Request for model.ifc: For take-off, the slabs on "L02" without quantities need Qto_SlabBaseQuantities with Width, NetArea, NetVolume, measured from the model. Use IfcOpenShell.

First a look at what the model holds.

```python
import ifcopenshell
import ifcopenshell.util.element
import ifcopenshell.util.unit

model = ifcopenshell.open("model.ifc")
print(model.schema)
for unit_type in ("LENGTHUNIT", "AREAUNIT", "VOLUMEUNIT"):
    print(unit_type, ifcopenshell.util.unit.calculate_unit_scale(model, unit_type))
storey = next(s for s in model.by_type("IfcBuildingStorey") if s.Name == "L02")
slabs = [e for e in ifcopenshell.util.element.get_decomposition(storey) if e.is_a("IfcSlab")]
for e in sorted(slabs, key=lambda e: e.id()):
    print(e.id(), e.is_a(), e.Name, list(ifcopenshell.util.element.get_psets(e, qtos_only=True)), sep=" | ")
```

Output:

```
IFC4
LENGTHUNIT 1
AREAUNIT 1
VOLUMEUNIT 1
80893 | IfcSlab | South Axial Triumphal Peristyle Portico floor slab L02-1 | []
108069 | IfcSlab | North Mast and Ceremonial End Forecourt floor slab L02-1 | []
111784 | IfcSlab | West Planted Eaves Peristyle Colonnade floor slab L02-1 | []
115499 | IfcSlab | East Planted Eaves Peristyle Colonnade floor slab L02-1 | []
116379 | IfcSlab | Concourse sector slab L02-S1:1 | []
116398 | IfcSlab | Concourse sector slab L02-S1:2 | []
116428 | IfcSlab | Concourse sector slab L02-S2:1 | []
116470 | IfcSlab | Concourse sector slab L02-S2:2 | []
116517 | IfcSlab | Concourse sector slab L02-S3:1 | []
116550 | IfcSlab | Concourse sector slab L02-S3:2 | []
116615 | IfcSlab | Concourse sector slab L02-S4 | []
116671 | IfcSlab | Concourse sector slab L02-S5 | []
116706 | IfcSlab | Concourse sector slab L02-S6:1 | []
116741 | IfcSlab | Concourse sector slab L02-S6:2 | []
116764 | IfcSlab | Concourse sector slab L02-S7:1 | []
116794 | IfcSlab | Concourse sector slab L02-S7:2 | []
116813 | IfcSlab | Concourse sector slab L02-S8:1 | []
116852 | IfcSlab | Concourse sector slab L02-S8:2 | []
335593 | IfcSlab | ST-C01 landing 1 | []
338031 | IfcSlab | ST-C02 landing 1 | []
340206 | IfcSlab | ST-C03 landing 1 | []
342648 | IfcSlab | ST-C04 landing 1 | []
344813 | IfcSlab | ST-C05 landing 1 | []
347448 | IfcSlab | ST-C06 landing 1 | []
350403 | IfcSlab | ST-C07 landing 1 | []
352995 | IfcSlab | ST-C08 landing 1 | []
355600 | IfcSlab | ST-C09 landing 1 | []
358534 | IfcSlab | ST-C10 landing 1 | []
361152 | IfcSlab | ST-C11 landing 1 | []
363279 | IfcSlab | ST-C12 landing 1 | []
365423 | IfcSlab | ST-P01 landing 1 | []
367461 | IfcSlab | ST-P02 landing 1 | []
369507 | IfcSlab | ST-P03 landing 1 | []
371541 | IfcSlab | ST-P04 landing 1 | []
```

```python
import ifcopenshell
import ifcopenshell.api.pset
import ifcopenshell.geom
import ifcopenshell.util.element
import ifcopenshell.util.shape
import ifcopenshell.util.unit

model = ifcopenshell.open("model.ifc")
unit_scale = ifcopenshell.util.unit.calculate_unit_scale(model)
area_scale = ifcopenshell.util.unit.calculate_unit_scale(model, "AREAUNIT")
volume_scale = ifcopenshell.util.unit.calculate_unit_scale(model, "VOLUMEUNIT")
settings = ifcopenshell.geom.settings()

storey = next(s for s in model.by_type("IfcBuildingStorey") if s.Name == "L02")
slabs = [e for e in ifcopenshell.util.element.get_decomposition(storey) if e.is_a("IfcSlab")]

for e in sorted(slabs, key=lambda e: e.id()):
    if ifcopenshell.util.element.get_psets(e, qtos_only=True, should_inherit=False):
        continue
    # Geometry comes back in metres, in the element's own axes.
    shape = ifcopenshell.geom.create_shape(settings, e)
    values = {
        "Width": ifcopenshell.util.shape.get_z(shape.geometry) / unit_scale,
        "NetArea": ifcopenshell.util.shape.get_footprint_area(shape.geometry) / area_scale,
        "NetVolume": ifcopenshell.util.shape.get_volume(shape.geometry) / volume_scale,
    }
    qto = ifcopenshell.api.pset.add_qto(model, product=e, name="Qto_SlabBaseQuantities")
    ifcopenshell.api.pset.edit_qto(model, qto=qto, properties=values)
    print(e.id(), {k: round(v, 3) for k, v in values.items()})

model.write("model_edited.ifc")
```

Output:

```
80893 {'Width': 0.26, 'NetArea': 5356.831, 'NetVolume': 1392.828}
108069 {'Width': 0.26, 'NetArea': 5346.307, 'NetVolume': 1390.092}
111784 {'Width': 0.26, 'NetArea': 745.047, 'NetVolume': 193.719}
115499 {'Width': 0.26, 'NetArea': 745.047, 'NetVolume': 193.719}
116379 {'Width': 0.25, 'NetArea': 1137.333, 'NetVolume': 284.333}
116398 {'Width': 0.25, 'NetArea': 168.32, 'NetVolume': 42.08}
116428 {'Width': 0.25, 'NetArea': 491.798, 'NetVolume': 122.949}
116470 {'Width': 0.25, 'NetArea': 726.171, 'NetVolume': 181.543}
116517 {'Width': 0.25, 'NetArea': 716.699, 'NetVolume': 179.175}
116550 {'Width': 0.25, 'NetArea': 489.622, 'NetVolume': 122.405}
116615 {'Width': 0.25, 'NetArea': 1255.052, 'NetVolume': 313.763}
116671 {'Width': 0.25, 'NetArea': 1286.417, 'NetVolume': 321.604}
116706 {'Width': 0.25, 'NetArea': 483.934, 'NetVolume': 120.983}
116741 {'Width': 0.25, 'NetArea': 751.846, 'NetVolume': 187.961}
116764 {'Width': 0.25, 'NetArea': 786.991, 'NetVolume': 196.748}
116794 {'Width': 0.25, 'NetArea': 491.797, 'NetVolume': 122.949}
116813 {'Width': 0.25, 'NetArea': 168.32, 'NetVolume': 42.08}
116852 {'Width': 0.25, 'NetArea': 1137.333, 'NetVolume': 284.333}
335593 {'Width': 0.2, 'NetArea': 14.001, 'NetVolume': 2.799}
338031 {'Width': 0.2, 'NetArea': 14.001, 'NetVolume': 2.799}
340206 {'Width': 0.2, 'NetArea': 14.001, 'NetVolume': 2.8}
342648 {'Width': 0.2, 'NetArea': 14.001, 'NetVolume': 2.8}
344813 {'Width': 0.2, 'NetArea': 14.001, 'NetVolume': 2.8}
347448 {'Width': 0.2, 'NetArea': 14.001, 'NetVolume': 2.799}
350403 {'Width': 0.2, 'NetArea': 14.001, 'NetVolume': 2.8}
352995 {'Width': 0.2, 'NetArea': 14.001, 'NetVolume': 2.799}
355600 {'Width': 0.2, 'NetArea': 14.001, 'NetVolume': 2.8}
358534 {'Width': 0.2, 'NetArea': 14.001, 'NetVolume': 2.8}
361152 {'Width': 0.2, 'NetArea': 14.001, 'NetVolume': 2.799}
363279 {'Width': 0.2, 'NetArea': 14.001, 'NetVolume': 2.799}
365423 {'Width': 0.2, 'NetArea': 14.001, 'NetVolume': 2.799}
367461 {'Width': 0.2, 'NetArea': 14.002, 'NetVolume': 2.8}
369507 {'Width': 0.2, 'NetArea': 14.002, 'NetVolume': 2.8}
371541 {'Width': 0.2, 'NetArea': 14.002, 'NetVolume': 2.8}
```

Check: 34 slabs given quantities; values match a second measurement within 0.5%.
